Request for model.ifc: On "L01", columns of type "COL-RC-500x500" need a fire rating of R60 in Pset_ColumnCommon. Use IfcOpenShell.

First a look at what the model holds.

```python
import ifcopenshell
import ifcopenshell.util.element

model = ifcopenshell.open("model.ifc")
print(model.schema)
storey = next(s for s in model.by_type("IfcBuildingStorey") if s.Name == "L01")
columns = [e for e in ifcopenshell.util.element.get_decomposition(storey) if e.is_a("IfcColumn")]
seen = {}
for e in columns:
    element_type = ifcopenshell.util.element.get_type(e)
    key = (element_type.Name if element_type != e and element_type else None, ifcopenshell.util.element.get_pset(e, "Pset_ColumnCommon", "FireRating"))
    seen[key] = seen.get(key, 0) + 1
for (name, value), count in sorted(seen.items(), key=str):
    print(count, "x", name, "|", value)
```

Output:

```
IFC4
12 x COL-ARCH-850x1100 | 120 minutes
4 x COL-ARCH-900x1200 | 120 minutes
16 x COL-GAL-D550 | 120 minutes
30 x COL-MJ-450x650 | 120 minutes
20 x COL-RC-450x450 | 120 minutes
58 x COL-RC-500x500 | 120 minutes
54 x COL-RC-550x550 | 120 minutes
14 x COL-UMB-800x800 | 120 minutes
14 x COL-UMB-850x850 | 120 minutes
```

```python
import ifcopenshell
import ifcopenshell.api.pset
import ifcopenshell.util.element

model = ifcopenshell.open("model.ifc")

storey = next(s for s in model.by_type("IfcBuildingStorey") if s.Name == "L01")
columns = [e for e in ifcopenshell.util.element.get_decomposition(storey) if e.is_a("IfcColumn")]

count = 0
for e in columns:
    element_type = ifcopenshell.util.element.get_type(e)
    if element_type in (None, e) or element_type.Name != "COL-RC-500x500":
        continue
    # add_pset returns the element's existing set when there is one.
    pset = ifcopenshell.api.pset.add_pset(model, product=e, name="Pset_ColumnCommon")
    ifcopenshell.api.pset.edit_pset(model, pset=pset, properties={"FireRating": "R60"})
    count += 1

print(count, "columns updated")

model.write("model_v2.ifc")
```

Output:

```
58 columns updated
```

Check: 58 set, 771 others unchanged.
